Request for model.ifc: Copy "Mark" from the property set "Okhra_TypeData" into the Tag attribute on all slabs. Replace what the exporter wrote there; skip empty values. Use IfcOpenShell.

First a look at what the model holds.

```python
import ifcopenshell
import ifcopenshell.util.element

model = ifcopenshell.open("model.ifc")
print(model.schema)
slabs = model.by_type("IfcSlab")
print(len(slabs), "slabs")
for e in slabs[:8]:
    source = ifcopenshell.util.element.get_pset(e, "Okhra_TypeData", "Mark")
    target = e.Tag
    print(e.id(), repr(source), repr(target), sep=" | ")
```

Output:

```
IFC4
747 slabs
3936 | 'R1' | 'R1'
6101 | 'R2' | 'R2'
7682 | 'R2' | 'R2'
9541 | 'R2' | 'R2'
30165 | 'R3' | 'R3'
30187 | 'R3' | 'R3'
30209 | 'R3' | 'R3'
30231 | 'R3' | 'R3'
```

```python
import ifcopenshell
import ifcopenshell.util.element

model = ifcopenshell.open("model.ifc")

count = 0
for e in model.by_type("IfcSlab"):
    value = ifcopenshell.util.element.get_pset(e, "Okhra_TypeData", "Mark")
    current = e.Tag
    if not value or not value.strip() or current == value:
        continue
    e.Tag = value
    count += 1

print(count, "slabs updated")

model.write("model_edited.ifc")
```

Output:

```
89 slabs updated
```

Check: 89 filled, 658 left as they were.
